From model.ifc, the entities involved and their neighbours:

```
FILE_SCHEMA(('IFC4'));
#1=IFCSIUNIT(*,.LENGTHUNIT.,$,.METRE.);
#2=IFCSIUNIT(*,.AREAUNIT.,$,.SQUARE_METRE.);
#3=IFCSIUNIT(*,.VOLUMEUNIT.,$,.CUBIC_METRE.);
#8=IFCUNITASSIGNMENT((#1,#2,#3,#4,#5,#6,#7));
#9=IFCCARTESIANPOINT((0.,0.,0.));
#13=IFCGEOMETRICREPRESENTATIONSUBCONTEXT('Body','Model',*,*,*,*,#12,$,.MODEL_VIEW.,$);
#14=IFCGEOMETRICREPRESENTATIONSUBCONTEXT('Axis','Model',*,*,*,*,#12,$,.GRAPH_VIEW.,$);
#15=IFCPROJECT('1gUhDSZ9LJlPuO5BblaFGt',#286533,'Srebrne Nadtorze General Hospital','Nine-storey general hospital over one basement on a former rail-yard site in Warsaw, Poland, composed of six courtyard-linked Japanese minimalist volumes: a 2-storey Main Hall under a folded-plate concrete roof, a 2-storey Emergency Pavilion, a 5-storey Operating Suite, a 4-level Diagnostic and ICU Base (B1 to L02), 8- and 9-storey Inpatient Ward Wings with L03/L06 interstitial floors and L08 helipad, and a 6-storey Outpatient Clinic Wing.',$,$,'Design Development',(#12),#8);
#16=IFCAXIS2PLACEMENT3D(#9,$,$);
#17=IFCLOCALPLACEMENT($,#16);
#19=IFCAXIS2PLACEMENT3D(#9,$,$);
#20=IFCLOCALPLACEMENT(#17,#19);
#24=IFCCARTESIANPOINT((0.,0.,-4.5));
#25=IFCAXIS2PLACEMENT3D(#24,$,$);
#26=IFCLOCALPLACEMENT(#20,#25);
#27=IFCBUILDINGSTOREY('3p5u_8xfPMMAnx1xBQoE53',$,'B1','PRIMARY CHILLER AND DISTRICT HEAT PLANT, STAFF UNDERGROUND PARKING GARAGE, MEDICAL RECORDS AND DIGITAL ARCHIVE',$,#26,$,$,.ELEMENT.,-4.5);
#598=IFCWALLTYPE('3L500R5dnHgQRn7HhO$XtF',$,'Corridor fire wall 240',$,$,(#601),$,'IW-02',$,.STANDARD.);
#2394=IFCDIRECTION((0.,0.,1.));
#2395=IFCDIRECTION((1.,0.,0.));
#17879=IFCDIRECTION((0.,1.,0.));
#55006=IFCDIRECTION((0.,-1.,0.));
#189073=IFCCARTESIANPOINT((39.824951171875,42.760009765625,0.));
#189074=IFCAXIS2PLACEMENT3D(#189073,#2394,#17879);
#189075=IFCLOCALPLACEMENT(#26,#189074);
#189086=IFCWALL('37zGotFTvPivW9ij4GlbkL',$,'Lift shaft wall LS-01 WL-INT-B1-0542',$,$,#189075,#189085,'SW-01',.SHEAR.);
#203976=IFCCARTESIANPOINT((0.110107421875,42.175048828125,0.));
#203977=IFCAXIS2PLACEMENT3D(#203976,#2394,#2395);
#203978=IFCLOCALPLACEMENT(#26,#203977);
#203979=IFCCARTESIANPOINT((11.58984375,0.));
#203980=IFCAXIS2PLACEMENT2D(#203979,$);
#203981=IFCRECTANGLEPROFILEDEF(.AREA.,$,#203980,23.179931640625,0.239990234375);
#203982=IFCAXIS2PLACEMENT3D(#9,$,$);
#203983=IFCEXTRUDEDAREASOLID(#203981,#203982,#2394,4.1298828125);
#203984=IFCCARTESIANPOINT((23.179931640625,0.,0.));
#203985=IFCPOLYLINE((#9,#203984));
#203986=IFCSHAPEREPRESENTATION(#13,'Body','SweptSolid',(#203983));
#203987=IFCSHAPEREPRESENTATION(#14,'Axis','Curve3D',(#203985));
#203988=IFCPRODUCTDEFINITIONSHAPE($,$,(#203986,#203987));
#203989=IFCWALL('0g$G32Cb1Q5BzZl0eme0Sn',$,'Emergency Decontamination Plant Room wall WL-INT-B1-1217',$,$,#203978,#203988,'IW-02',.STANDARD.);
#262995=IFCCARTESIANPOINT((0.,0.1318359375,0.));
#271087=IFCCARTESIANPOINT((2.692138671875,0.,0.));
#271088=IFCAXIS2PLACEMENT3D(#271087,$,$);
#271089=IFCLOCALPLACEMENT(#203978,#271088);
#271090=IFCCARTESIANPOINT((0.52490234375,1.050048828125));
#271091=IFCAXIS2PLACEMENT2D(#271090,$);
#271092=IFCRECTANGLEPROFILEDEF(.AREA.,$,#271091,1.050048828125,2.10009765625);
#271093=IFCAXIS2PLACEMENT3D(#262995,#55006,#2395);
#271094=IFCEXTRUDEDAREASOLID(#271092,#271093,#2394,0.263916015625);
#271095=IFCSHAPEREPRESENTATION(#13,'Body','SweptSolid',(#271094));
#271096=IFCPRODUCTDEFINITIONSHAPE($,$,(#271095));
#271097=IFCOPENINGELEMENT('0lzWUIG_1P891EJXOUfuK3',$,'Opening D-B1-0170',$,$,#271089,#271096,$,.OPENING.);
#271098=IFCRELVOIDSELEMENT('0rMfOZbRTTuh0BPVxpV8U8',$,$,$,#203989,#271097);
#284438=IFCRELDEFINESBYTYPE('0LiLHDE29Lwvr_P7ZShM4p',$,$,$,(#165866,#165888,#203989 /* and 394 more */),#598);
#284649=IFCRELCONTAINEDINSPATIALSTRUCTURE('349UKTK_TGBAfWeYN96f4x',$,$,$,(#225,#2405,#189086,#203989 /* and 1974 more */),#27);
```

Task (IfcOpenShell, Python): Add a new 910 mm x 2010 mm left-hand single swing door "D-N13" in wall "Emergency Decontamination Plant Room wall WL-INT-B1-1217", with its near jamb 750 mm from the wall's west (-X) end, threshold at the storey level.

```python
import numpy as np
import ifcopenshell
import ifcopenshell.api.feature
import ifcopenshell.api.geometry
import ifcopenshell.api.root
import ifcopenshell.api.spatial
import ifcopenshell.geom
import ifcopenshell.util.element
import ifcopenshell.util.placement
import ifcopenshell.util.representation
import ifcopenshell.util.shape
import ifcopenshell.util.unit

model = ifcopenshell.open("model.ifc")
unit_scale = ifcopenshell.util.unit.calculate_unit_scale(model)
settings = ifcopenshell.geom.settings()


def volume(element):
    """Net volume in cubic metres, openings subtracted."""
    shape = ifcopenshell.geom.create_shape(settings, element)
    return ifcopenshell.util.shape.get_volume(shape.geometry)


wall = model.by_guid("0g$G32Cb1Q5BzZl0eme0Sn")
storey = ifcopenshell.util.element.get_container(wall, ifc_class="IfcBuildingStorey")
context = ifcopenshell.util.representation.get_context(model, "Model", "Body", "MODEL_VIEW")
before = volume(wall)

width, height, from_end, sill = 0.91, 2.01, 0.75, 0.0  # metres

# The wall runs along its own X axis, and the end named is its -X end.
wall_shape = ifcopenshell.geom.create_shape(settings, wall)
x, y, z = ifcopenshell.util.shape.get_vertices(wall_shape.geometry).T
start = x.min() + from_end
face, thickness = float(y.min()), float(y.max() - y.min())
wall_matrix = ifcopenshell.util.placement.get_local_placement(wall.ObjectPlacement)
level = ifcopenshell.util.placement.get_local_placement(storey.ObjectPlacement)[2, 3]


def in_wall(x, y):
    """Placement at x, y metres in the wall's axes, at sill height."""
    matrix = wall_matrix.copy()
    matrix[:, 3] = wall_matrix @ np.array([x / unit_scale, y / unit_scale, 0.0, 1.0])
    matrix[2, 3] = level + sill / unit_scale
    return matrix


# Opening: a box that overshoots both wall faces by 50 mm.
opening = ifcopenshell.api.root.create_entity(model, ifc_class="IfcOpeningElement", predefined_type="OPENING")
box = ifcopenshell.api.geometry.add_wall_representation(
    model, context=context, length=width, height=height, thickness=thickness + 0.1
)
ifcopenshell.api.geometry.assign_representation(model, product=opening, representation=box)
ifcopenshell.api.geometry.edit_object_placement(model, product=opening, matrix=in_wall(start, face - 0.05), is_si=False)
ifcopenshell.api.feature.add_feature(model, feature=opening, element=wall)

door = ifcopenshell.api.root.create_entity(model, ifc_class="IfcDoor", name="D-N13", predefined_type="DOOR")
door.OverallWidth, door.OverallHeight = width / unit_scale, height / unit_scale
door.OperationType = "SINGLE_SWING_LEFT"
body = ifcopenshell.api.geometry.add_door_representation(
    model,
    context=context,
    overall_width=door.OverallWidth,
    overall_height=door.OverallHeight,
    operation_type="SINGLE_SWING_LEFT",
    lining_properties={"LiningDepth": thickness / unit_scale, "ThresholdDepth": thickness / unit_scale},
)
ifcopenshell.api.geometry.assign_representation(model, product=door, representation=body)
ifcopenshell.api.spatial.assign_container(model, products=[door], relating_structure=storey)
ifcopenshell.api.feature.add_filling(model, opening=opening, element=door)

# The lining spans the wall, so the door starts at the wall face.
ifcopenshell.api.geometry.edit_object_placement(model, product=door, matrix=in_wall(start, face), is_si=False)

after = volume(wall)

print(f"wall volume {before:.3f} -> {after:.3f} m3")

model.write("model_v2.ifc")
```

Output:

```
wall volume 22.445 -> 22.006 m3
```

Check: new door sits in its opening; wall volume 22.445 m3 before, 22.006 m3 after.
